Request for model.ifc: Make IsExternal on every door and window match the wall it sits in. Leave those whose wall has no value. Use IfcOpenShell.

First a look at what the model holds.

```python
import ifcopenshell
import ifcopenshell.util.element

model = ifcopenshell.open("model.ifc")
print(model.schema)
seen = {}
for e in model.by_type("IfcDoor") + model.by_type("IfcWindow"):
    if not e.FillsVoids:
        continue
    host = e.FillsVoids[0].RelatingOpeningElement.VoidsElements[0].RelatingBuildingElement
    own = ifcopenshell.util.element.get_pset(e, f"Pset_{e.is_a()[3:].removesuffix('StandardCase')}Common", "IsExternal")
    wall = ifcopenshell.util.element.get_pset(host, "Pset_WallCommon", "IsExternal")
    seen[e.is_a(), own, wall] = seen.get((e.is_a(), own, wall), 0) + 1
for (cls, own, wall), count in sorted(seen.items(), key=str):
    print(count, cls, "IsExternal:", own, "| host wall:", wall)
```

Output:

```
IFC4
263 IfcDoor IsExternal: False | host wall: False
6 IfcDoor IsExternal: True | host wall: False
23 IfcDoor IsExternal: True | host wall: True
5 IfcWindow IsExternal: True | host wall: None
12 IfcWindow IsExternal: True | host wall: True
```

```python
import ifcopenshell
import ifcopenshell.api.pset
import ifcopenshell.util.element

model = ifcopenshell.open("model.ifc")

count = 0
for ifc_class, pset_name in (("IfcDoor", "Pset_DoorCommon"), ("IfcWindow", "Pset_WindowCommon")):
    for e in model.by_type(ifc_class):
        if not e.FillsVoids:
            continue
        host = e.FillsVoids[0].RelatingOpeningElement.VoidsElements[0].RelatingBuildingElement
        external = ifcopenshell.util.element.get_pset(host, "Pset_WallCommon", "IsExternal")
        if external is None or ifcopenshell.util.element.get_pset(e, pset_name, "IsExternal") == external:
            continue
        pset = ifcopenshell.api.pset.add_pset(model, product=e, name=pset_name)
        ifcopenshell.api.pset.edit_pset(model, pset=pset, properties={"IsExternal": external})
        count += 1

print(count, "updated")

model.write("model_v2.ifc")
```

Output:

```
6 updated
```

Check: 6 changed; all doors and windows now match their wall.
